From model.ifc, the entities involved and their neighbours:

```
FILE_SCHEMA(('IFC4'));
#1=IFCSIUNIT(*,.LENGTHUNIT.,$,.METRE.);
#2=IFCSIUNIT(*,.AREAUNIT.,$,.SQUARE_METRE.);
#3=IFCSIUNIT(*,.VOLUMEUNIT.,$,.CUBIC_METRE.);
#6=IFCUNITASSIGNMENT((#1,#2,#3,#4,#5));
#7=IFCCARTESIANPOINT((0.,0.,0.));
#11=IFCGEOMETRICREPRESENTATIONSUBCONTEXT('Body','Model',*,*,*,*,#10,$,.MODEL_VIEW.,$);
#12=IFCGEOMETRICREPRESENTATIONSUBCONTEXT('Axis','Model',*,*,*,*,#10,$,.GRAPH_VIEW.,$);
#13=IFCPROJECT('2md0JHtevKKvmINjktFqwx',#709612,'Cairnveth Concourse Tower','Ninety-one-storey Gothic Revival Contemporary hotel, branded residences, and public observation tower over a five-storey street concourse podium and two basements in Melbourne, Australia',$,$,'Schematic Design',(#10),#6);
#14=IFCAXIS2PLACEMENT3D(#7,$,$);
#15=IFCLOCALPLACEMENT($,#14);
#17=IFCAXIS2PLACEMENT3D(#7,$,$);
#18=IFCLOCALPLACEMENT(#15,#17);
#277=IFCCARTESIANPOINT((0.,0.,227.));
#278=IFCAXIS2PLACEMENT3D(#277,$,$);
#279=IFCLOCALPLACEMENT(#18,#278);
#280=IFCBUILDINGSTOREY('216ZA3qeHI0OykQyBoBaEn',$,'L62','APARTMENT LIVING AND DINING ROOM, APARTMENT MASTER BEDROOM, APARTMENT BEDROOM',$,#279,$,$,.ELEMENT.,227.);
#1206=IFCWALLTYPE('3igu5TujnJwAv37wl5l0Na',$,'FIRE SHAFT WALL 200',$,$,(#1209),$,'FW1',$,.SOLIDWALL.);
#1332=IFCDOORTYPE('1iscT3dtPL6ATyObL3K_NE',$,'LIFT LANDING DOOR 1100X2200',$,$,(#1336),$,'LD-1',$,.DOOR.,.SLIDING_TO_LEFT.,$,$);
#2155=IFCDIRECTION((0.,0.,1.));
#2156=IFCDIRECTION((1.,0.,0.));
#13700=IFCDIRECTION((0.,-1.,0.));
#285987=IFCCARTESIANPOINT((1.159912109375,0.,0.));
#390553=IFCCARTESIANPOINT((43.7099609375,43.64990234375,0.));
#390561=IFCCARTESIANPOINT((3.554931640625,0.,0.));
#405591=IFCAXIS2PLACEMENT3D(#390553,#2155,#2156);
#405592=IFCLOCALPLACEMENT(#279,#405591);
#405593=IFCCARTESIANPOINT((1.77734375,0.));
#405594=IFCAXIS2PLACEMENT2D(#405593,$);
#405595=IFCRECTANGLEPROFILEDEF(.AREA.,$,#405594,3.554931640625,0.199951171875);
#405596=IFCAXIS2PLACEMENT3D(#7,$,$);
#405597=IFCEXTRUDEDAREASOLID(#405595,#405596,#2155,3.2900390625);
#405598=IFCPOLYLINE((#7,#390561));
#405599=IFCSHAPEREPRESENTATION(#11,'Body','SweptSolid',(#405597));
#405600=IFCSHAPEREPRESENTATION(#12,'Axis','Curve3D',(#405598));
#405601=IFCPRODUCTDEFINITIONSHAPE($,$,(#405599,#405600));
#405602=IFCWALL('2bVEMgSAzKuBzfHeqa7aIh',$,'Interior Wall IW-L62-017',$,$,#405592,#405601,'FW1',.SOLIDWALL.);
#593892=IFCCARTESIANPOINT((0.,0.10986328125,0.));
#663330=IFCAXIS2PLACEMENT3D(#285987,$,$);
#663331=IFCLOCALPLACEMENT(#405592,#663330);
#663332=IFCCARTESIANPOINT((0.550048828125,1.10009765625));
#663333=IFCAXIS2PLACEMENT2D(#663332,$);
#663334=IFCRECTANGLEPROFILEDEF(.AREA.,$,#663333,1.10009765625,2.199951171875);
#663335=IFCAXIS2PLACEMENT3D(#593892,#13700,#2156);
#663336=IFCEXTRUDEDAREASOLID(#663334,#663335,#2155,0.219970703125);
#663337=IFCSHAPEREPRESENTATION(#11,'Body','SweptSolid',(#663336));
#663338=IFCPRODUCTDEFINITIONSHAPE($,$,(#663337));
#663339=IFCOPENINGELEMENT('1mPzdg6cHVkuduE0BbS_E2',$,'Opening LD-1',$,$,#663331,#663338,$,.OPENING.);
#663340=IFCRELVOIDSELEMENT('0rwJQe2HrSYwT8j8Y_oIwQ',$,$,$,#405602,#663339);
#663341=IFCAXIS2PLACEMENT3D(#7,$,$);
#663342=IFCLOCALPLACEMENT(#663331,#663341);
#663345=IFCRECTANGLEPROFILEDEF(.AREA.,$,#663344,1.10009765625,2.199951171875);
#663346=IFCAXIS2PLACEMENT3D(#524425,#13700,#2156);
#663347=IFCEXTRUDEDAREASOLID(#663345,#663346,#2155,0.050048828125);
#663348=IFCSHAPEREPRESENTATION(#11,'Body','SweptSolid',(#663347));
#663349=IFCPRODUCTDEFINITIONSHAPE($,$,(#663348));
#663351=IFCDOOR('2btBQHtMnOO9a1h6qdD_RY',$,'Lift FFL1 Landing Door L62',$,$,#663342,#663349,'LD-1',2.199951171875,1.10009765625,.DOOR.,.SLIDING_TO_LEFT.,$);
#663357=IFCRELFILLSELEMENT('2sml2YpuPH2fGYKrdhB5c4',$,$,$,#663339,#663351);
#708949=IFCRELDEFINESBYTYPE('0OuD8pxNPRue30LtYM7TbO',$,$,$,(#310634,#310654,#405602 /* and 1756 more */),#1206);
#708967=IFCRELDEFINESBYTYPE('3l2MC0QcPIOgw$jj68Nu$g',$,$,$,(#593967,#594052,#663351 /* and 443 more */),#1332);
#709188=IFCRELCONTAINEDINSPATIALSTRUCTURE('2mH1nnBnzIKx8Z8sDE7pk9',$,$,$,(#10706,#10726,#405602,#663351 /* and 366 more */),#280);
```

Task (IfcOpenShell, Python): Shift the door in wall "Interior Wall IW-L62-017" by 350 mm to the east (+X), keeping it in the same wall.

```python
import ifcopenshell
import ifcopenshell.api.geometry
import ifcopenshell.util.placement

model = ifcopenshell.open("model.ifc")

door = model.by_id(663351)
opening = door.FillsVoids[0].RelatingOpeningElement
wall = opening.VoidsElements[0].RelatingBuildingElement

wall_matrix = ifcopenshell.util.placement.get_local_placement(wall.ObjectPlacement)
shift = wall_matrix[:3, 0] * 0.35
before = ifcopenshell.util.placement.get_local_placement(door.ObjectPlacement)[:3, 3].copy()

# The door is placed relative to its opening, so it follows when the opening moves.
matrix = ifcopenshell.util.placement.get_local_placement(opening.ObjectPlacement)
matrix[:3, 3] += shift
ifcopenshell.api.geometry.edit_object_placement(
    model, product=opening, matrix=matrix, is_si=False, should_transform_children=True
)

after = ifcopenshell.util.placement.get_local_placement(door.ObjectPlacement)[:3, 3]
print("door moved by", (after - before).round(3) + 0.0)

model.write("model_updated.ifc")
```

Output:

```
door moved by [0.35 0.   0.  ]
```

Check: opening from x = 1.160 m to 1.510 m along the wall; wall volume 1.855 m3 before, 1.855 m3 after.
